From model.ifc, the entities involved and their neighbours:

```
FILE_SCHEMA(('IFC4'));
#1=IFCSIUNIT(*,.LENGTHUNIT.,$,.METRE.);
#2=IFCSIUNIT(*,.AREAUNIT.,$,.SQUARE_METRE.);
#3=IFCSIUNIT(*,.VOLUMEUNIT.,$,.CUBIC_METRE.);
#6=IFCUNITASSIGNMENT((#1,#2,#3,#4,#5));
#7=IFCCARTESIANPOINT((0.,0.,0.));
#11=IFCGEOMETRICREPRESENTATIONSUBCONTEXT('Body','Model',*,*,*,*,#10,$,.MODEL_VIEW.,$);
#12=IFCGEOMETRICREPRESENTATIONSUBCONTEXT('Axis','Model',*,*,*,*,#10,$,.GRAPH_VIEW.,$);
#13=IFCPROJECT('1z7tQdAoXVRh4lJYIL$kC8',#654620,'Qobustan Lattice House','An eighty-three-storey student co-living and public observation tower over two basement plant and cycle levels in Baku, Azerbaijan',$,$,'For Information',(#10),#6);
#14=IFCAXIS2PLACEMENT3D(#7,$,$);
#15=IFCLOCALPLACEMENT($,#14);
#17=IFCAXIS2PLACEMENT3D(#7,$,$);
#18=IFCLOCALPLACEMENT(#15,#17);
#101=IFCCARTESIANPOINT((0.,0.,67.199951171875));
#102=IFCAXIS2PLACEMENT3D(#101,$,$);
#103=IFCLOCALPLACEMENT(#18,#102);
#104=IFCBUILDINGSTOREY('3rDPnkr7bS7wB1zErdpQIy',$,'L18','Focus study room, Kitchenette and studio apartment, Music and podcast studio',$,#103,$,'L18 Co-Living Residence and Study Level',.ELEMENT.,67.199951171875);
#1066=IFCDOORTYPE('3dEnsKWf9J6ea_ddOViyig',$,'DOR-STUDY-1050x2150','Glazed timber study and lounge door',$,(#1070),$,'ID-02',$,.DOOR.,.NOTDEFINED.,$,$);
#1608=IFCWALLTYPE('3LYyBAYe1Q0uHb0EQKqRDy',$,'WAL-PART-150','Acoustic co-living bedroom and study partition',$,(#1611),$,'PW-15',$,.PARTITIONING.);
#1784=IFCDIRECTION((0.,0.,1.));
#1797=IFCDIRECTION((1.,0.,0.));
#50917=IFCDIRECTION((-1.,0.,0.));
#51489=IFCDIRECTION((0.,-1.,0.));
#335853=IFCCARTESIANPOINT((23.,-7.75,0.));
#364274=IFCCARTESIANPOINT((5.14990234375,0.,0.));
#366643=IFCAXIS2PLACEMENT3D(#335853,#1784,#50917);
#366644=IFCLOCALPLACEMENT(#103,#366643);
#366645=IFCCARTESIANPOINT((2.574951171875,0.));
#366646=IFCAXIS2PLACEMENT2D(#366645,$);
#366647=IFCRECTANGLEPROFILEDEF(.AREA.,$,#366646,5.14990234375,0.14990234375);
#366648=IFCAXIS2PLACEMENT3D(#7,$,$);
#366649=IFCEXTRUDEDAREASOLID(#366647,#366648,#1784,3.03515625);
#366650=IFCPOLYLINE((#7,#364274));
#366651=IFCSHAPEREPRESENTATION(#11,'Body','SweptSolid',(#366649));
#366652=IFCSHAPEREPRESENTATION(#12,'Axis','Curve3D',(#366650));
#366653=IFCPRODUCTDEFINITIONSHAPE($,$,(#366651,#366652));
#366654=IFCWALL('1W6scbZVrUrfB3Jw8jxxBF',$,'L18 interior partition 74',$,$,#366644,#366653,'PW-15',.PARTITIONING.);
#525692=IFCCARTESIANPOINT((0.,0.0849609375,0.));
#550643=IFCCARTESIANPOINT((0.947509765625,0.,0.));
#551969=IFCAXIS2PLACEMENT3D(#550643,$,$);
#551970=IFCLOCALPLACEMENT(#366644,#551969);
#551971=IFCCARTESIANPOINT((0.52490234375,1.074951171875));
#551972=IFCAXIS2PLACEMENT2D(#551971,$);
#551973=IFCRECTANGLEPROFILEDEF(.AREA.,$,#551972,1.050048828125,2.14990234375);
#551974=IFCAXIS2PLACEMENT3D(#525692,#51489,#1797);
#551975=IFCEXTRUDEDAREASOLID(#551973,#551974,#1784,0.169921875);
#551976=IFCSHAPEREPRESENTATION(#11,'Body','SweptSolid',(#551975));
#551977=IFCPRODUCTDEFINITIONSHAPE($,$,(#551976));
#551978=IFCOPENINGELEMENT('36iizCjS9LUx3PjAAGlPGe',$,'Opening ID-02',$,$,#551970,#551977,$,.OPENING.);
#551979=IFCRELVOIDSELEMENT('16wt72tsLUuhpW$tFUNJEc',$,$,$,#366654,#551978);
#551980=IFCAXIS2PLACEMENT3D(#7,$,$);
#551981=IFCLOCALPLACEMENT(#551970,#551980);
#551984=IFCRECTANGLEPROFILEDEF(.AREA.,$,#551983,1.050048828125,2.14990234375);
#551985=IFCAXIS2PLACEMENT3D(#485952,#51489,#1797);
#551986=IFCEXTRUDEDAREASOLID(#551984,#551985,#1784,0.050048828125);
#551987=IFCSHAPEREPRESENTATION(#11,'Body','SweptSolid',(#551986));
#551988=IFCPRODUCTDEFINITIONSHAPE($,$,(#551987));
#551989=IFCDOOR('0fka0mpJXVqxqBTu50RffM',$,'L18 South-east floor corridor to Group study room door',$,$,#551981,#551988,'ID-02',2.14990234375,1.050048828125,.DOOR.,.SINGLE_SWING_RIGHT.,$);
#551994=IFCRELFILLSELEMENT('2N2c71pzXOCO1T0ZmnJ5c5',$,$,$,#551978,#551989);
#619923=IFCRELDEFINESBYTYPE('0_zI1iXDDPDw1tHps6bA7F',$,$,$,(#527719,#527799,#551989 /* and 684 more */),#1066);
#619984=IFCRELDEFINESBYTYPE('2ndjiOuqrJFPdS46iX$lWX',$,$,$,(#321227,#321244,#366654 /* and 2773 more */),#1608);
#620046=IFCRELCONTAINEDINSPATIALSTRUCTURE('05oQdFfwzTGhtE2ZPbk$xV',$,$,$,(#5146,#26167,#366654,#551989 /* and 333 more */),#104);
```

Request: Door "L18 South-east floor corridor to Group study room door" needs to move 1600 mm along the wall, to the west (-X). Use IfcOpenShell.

```python
import ifcopenshell
import ifcopenshell.api.geometry
import ifcopenshell.util.placement

model = ifcopenshell.open("model.ifc")

door = model.by_guid("0fka0mpJXVqxqBTu50RffM")
opening = door.FillsVoids[0].RelatingOpeningElement
wall = opening.VoidsElements[0].RelatingBuildingElement

wall_matrix = ifcopenshell.util.placement.get_local_placement(wall.ObjectPlacement)
shift = wall_matrix[:3, 0] * 1.6
before = ifcopenshell.util.placement.get_local_placement(door.ObjectPlacement)[:3, 3].copy()

# The door is placed relative to its opening, so it follows when the opening moves.
matrix = ifcopenshell.util.placement.get_local_placement(opening.ObjectPlacement)
matrix[:3, 3] += shift
ifcopenshell.api.geometry.edit_object_placement(
    model, product=opening, matrix=matrix, is_si=False, should_transform_children=True
)

after = ifcopenshell.util.placement.get_local_placement(door.ObjectPlacement)[:3, 3]
print("door moved by", (after - before).round(3) + 0.0)

model.write("model-out.ifc")
```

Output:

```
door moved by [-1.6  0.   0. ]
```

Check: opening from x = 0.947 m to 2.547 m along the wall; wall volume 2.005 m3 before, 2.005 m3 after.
